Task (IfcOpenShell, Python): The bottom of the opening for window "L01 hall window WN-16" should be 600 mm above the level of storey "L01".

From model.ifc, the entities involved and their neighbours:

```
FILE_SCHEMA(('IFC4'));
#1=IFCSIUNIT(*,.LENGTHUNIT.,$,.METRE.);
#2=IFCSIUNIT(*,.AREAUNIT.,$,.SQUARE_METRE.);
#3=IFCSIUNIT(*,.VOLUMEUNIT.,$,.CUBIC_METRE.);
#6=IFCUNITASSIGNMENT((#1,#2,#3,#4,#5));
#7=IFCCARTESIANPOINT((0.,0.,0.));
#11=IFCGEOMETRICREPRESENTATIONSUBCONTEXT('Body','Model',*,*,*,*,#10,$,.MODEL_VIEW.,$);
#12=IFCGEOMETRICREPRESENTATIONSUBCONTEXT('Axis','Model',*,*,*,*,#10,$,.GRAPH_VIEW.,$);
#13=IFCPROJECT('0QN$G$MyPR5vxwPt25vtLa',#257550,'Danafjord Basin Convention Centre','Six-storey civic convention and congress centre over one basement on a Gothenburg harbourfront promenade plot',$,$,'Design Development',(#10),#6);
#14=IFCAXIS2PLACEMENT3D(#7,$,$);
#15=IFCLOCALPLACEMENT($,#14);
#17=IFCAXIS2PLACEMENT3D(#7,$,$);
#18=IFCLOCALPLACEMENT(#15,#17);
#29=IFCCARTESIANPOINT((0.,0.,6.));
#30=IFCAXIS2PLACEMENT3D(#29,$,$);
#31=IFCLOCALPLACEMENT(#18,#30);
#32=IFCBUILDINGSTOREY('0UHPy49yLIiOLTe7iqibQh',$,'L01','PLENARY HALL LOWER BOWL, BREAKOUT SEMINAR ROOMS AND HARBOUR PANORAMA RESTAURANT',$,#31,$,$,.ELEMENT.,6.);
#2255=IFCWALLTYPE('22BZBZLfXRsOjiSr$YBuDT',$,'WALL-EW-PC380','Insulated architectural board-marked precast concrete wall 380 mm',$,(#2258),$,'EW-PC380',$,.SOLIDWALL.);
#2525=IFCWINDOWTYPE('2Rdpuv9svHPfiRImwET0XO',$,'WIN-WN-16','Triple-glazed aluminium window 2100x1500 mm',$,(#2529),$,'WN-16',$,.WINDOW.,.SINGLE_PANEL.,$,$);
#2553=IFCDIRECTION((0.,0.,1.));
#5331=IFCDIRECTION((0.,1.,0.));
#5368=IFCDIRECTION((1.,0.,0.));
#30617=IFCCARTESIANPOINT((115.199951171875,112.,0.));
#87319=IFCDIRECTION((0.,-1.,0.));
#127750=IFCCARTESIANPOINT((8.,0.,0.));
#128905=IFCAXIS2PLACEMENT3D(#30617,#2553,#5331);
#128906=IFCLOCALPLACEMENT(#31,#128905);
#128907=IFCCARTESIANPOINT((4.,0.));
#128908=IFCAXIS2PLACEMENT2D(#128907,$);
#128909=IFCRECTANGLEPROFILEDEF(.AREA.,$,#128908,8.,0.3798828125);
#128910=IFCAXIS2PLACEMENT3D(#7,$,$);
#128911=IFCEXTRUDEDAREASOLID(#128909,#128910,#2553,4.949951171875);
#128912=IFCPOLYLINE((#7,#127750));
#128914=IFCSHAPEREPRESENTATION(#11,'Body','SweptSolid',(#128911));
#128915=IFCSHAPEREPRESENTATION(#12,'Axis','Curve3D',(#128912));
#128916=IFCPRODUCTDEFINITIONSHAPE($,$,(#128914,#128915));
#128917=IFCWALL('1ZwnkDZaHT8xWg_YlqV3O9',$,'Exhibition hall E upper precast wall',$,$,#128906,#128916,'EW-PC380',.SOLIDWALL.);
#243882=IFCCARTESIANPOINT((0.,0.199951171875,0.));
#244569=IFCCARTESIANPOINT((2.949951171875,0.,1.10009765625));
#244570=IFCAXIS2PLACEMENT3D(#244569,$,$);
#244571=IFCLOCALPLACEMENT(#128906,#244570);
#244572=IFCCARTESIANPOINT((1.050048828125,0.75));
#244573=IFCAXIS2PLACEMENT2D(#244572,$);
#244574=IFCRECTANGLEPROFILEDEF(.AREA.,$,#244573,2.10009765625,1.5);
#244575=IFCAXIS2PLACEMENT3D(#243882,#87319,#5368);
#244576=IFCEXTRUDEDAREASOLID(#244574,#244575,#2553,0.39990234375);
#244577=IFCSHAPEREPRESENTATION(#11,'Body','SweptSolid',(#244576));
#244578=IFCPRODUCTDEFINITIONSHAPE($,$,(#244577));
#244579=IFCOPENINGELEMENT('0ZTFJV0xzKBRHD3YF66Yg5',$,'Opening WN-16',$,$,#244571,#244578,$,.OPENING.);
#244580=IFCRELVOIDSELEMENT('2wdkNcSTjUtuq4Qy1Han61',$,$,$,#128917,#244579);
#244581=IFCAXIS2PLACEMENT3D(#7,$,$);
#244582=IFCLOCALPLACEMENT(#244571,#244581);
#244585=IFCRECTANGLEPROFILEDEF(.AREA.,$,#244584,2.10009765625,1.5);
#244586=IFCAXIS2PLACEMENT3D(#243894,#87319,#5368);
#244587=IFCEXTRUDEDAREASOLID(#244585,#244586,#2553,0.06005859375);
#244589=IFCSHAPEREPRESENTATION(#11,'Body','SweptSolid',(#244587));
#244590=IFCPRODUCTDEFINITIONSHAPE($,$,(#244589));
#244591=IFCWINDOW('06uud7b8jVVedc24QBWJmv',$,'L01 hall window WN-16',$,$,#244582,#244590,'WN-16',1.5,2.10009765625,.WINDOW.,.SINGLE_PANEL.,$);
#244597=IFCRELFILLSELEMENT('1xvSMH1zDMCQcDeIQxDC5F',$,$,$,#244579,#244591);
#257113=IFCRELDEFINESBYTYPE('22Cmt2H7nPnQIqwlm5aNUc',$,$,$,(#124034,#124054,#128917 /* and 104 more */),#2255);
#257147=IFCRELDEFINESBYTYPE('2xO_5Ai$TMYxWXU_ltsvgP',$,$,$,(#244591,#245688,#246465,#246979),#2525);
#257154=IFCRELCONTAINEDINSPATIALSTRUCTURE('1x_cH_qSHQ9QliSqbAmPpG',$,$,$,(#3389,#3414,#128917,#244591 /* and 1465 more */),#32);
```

```python
import numpy as np
import ifcopenshell
import ifcopenshell.api.geometry
import ifcopenshell.geom
import ifcopenshell.util.element
import ifcopenshell.util.placement
import ifcopenshell.util.shape
import ifcopenshell.util.unit

model = ifcopenshell.open("model.ifc")
unit_scale = ifcopenshell.util.unit.calculate_unit_scale(model)

window = model.by_guid("06uud7b8jVVedc24QBWJmv")
opening = window.FillsVoids[0].RelatingOpeningElement
storey = ifcopenshell.util.element.get_container(window, ifc_class="IfcBuildingStorey")
level = ifcopenshell.util.placement.get_local_placement(storey.ObjectPlacement)[2, 3]

# The opening's origin need not be at the sill, so measure its lowest point.
shape = ifcopenshell.geom.create_shape(ifcopenshell.geom.settings(), opening)
bottom = ifcopenshell.util.shape.get_shape_bottom_elevation(shape, shape.geometry) / unit_scale
dz = level + 0.6 / unit_scale - bottom

shift = np.array([0.0, 0.0, dz])
# The window is placed relative to its opening, so it follows when the opening moves.
matrix = ifcopenshell.util.placement.get_local_placement(opening.ObjectPlacement)
matrix[:3, 3] += shift
ifcopenshell.api.geometry.edit_object_placement(
    model, product=opening, matrix=matrix, is_si=False, should_transform_children=True
)

print(f"moved by {dz * unit_scale:+.3f} m")

model.write("model_updated.ifc")
```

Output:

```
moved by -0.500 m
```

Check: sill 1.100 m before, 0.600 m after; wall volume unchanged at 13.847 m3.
